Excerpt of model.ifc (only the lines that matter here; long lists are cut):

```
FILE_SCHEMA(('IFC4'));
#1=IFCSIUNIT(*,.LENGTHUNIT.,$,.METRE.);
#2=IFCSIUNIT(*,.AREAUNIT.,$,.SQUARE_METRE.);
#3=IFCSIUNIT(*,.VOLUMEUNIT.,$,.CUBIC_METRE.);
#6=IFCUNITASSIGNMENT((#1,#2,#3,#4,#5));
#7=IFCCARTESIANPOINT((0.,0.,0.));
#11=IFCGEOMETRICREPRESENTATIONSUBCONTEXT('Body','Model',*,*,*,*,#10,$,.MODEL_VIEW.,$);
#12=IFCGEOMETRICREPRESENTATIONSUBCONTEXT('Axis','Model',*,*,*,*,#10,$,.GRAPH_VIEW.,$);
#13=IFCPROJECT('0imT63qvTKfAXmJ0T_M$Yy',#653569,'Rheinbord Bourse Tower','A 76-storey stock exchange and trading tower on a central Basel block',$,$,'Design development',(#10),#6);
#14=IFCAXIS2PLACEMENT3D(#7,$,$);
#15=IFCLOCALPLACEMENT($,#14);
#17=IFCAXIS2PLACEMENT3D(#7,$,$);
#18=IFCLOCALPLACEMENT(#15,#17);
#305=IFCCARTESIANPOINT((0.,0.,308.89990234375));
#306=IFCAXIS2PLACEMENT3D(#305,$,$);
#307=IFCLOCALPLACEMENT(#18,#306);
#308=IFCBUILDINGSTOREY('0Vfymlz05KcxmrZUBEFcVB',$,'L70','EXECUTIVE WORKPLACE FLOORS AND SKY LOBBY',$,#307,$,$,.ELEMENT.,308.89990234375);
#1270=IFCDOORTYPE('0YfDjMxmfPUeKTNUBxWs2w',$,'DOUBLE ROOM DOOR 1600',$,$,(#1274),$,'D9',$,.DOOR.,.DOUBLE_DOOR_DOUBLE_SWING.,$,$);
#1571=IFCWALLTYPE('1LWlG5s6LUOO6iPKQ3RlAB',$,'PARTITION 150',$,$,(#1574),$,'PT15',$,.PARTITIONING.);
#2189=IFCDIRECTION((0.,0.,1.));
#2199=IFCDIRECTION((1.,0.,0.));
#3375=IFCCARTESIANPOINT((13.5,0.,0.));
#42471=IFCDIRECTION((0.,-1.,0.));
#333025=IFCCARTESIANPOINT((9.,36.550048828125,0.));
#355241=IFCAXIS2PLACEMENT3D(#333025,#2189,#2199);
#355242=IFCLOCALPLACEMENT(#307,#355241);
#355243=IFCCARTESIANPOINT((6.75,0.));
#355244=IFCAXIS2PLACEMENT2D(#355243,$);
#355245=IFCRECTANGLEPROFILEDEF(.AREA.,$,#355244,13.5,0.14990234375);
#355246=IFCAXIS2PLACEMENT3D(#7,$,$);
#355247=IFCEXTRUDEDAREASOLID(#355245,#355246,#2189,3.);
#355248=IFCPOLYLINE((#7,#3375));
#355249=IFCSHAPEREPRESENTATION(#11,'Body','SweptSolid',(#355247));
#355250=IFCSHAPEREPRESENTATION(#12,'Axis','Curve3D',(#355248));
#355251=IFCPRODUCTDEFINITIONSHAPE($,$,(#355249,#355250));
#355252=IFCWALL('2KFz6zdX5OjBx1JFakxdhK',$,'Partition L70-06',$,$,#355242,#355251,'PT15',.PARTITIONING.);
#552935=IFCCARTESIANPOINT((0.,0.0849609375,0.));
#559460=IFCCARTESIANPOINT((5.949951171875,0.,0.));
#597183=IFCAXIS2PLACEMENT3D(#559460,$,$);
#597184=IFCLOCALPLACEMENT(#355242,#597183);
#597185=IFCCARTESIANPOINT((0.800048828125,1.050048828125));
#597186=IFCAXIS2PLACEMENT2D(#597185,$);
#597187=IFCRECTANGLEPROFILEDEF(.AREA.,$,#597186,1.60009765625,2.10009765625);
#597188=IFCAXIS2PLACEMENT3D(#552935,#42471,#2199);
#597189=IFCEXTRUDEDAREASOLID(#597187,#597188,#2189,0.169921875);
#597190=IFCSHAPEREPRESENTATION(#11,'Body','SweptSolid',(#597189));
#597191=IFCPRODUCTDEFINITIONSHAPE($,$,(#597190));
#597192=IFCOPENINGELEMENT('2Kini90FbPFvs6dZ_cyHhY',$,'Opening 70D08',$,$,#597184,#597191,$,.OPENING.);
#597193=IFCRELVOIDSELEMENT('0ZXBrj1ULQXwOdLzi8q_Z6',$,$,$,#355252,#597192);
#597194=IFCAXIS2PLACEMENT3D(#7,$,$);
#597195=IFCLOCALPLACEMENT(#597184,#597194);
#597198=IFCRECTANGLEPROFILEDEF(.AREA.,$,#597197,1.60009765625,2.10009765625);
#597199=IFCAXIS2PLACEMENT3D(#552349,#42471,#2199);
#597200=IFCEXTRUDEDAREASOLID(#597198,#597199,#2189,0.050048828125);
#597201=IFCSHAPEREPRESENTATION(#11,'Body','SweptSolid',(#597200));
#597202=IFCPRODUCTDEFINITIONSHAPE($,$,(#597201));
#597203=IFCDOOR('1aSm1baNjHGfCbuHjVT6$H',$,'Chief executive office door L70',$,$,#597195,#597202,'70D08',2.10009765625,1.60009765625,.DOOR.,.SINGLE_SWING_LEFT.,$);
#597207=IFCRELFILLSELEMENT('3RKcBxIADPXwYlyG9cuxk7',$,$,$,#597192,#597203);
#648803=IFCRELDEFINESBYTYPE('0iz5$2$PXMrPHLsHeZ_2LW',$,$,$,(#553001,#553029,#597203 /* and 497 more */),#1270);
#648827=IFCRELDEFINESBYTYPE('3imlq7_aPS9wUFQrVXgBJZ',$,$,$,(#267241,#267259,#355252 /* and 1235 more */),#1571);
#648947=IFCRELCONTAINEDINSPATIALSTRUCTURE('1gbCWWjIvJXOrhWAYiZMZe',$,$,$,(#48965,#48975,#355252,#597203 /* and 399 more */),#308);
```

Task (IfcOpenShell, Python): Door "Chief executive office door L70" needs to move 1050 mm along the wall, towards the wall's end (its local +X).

```python
import ifcopenshell
import ifcopenshell.api.geometry
import ifcopenshell.util.placement
import ifcopenshell.util.unit

model = ifcopenshell.open("model.ifc")
unit_scale = ifcopenshell.util.unit.calculate_unit_scale(model)

door = model.by_guid("1aSm1baNjHGfCbuHjVT6$H")
opening = door.FillsVoids[0].RelatingOpeningElement
wall = opening.VoidsElements[0].RelatingBuildingElement

wall_matrix = ifcopenshell.util.placement.get_local_placement(wall.ObjectPlacement)
shift = wall_matrix[:3, 0] * 1.05 / unit_scale
before = ifcopenshell.util.placement.get_local_placement(door.ObjectPlacement)[:3, 3].copy()

# The door is placed relative to its opening, so it follows when the opening moves.
matrix = ifcopenshell.util.placement.get_local_placement(opening.ObjectPlacement)
matrix[:3, 3] += shift
ifcopenshell.api.geometry.edit_object_placement(
    model, product=opening, matrix=matrix, is_si=False, should_transform_children=True
)

after = ifcopenshell.util.placement.get_local_placement(door.ObjectPlacement)[:3, 3]
print("door moved by", (after - before).round(3) + 0.0)

model.write("model_v2.ifc")
```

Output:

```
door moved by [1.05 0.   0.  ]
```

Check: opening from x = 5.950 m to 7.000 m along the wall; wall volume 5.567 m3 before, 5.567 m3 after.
